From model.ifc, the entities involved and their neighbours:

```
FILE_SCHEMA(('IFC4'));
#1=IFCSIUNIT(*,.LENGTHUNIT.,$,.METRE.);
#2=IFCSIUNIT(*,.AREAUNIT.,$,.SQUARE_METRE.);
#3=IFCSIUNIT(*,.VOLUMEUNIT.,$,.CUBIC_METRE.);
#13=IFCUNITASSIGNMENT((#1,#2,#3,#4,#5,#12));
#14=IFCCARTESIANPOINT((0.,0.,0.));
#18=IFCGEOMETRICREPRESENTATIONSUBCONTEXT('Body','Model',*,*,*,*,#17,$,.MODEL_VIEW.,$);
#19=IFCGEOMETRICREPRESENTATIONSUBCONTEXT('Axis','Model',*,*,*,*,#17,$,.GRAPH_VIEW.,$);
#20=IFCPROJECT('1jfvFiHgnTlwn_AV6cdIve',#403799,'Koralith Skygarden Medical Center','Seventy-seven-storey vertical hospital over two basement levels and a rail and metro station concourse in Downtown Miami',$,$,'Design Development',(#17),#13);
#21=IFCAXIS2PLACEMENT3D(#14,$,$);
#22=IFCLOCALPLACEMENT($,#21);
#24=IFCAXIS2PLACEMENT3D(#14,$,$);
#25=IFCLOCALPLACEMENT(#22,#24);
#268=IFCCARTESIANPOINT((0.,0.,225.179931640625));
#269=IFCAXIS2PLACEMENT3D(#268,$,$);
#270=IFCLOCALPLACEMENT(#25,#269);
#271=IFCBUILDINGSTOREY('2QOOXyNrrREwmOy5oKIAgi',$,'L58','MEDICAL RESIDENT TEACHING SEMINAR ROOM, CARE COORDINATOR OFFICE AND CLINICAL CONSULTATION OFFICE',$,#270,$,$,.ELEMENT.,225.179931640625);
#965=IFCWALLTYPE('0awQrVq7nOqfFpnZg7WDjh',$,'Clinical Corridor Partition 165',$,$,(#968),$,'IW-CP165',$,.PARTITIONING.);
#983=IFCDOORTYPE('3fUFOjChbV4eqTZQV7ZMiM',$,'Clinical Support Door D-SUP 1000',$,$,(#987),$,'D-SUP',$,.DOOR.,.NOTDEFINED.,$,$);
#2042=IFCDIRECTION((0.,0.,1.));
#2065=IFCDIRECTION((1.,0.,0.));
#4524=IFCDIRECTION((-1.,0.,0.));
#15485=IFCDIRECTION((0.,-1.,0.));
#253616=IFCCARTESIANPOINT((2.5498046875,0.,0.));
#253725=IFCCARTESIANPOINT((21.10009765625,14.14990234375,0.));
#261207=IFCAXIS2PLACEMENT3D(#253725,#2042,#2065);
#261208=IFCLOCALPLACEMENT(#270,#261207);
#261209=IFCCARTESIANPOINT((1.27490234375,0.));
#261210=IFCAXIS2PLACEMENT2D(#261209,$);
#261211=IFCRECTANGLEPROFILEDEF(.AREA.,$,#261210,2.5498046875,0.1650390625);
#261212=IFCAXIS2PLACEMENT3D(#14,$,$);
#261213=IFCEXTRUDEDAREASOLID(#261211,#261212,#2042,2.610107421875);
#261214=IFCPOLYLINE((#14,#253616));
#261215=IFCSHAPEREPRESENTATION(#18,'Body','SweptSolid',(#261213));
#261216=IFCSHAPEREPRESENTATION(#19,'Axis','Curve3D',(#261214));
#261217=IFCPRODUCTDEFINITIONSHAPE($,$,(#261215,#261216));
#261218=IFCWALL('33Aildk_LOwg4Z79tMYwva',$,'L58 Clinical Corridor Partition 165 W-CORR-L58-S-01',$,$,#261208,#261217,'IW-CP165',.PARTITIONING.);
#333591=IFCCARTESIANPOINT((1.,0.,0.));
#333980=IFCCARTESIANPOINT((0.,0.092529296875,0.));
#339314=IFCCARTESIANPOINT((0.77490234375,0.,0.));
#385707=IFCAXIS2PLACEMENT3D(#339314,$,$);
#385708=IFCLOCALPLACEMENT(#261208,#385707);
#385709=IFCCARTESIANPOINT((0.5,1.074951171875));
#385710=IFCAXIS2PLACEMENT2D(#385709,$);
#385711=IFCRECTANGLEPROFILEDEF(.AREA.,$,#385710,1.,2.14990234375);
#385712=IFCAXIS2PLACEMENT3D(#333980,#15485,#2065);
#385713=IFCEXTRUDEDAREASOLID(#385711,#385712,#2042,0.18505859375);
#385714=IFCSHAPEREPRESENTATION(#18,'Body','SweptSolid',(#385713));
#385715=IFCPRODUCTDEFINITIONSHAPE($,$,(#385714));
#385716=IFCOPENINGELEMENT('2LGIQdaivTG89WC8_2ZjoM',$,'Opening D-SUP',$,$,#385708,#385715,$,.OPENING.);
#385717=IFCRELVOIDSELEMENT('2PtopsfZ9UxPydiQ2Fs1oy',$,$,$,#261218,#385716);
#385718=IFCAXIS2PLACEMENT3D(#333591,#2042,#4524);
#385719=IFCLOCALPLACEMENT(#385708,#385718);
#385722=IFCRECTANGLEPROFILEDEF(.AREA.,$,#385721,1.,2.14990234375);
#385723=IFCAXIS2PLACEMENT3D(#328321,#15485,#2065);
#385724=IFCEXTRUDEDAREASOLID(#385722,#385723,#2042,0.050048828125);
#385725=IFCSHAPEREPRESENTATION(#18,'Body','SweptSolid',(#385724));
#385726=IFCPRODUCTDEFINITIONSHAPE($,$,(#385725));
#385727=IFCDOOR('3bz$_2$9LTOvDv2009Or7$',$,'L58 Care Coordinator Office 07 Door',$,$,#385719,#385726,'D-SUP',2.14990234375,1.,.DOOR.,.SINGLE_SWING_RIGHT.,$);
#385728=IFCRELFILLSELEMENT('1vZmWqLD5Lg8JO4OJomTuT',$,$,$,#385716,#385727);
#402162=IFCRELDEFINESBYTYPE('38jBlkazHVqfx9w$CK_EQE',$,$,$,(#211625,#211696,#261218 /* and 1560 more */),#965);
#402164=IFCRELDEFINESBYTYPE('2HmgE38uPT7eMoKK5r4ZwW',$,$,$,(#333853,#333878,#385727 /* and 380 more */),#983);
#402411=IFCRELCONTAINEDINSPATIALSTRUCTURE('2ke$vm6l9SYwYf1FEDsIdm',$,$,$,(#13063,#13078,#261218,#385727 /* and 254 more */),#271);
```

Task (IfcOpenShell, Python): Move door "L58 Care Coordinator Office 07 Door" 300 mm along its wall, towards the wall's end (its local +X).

```python
import ifcopenshell
import ifcopenshell.api.geometry
import ifcopenshell.util.placement
import ifcopenshell.util.unit

model = ifcopenshell.open("model.ifc")
unit_scale = ifcopenshell.util.unit.calculate_unit_scale(model)

door = model.by_id(385727)
opening = door.FillsVoids[0].RelatingOpeningElement
wall = opening.VoidsElements[0].RelatingBuildingElement

wall_matrix = ifcopenshell.util.placement.get_local_placement(wall.ObjectPlacement)
shift = wall_matrix[:3, 0] * 0.3 / unit_scale
before = ifcopenshell.util.placement.get_local_placement(door.ObjectPlacement)[:3, 3].copy()

# The door is placed relative to its opening, so it follows when the opening moves.
matrix = ifcopenshell.util.placement.get_local_placement(opening.ObjectPlacement)
matrix[:3, 3] += shift
ifcopenshell.api.geometry.edit_object_placement(
    model, product=opening, matrix=matrix, is_si=False, should_transform_children=True
)

after = ifcopenshell.util.placement.get_local_placement(door.ObjectPlacement)[:3, 3]
print("door moved by", (after - before).round(3) + 0.0)

model.write("model_rev.ifc")
```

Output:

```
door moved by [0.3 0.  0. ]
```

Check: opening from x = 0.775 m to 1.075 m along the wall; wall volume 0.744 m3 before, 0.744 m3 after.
